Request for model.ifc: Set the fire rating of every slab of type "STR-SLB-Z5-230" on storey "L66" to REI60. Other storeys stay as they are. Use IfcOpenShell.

First a look at what the model holds.

```python
import ifcopenshell
import ifcopenshell.util.element

model = ifcopenshell.open("model.ifc")
print(model.schema)
storey = next(s for s in model.by_type("IfcBuildingStorey") if s.Name == "L66")
slabs = [e for e in ifcopenshell.util.element.get_decomposition(storey) if e.is_a("IfcSlab")]
seen = {}
for e in slabs:
    element_type = ifcopenshell.util.element.get_type(e)
    key = (element_type.Name if element_type != e and element_type else None, ifcopenshell.util.element.get_pset(e, "Pset_SlabCommon", "FireRating"))
    seen[key] = seen.get(key, 0) + 1
for (name, value), count in sorted(seen.items(), key=str):
    print(count, "x", name, "|", value)
```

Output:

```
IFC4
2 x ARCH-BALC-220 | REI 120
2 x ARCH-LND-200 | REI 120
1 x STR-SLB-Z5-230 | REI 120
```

```python
import ifcopenshell
import ifcopenshell.api.pset
import ifcopenshell.util.element

model = ifcopenshell.open("model.ifc")

storey = next(s for s in model.by_type("IfcBuildingStorey") if s.Name == "L66")
slabs = [e for e in ifcopenshell.util.element.get_decomposition(storey) if e.is_a("IfcSlab")]

count = 0
for e in slabs:
    element_type = ifcopenshell.util.element.get_type(e)
    if element_type in (None, e) or element_type.Name != "STR-SLB-Z5-230":
        continue
    found = ifcopenshell.util.element.get_pset(e, "Pset_SlabCommon", should_inherit=False)
    if found:
        pset = model.by_id(found["id"])
        if len(ifcopenshell.util.element.get_elements_by_pset(pset)) > 1:
            pset = ifcopenshell.api.pset.unshare_pset(model, products=[e], pset=pset)[0]
    else:
        pset = ifcopenshell.api.pset.add_pset(model, product=e, name="Pset_SlabCommon")
    ifcopenshell.api.pset.edit_pset(model, pset=pset, properties={"FireRating": "REI60"})
    count += 1

print(count, "slabs updated")

model.write("model-out.ifc")
```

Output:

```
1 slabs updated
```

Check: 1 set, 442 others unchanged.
